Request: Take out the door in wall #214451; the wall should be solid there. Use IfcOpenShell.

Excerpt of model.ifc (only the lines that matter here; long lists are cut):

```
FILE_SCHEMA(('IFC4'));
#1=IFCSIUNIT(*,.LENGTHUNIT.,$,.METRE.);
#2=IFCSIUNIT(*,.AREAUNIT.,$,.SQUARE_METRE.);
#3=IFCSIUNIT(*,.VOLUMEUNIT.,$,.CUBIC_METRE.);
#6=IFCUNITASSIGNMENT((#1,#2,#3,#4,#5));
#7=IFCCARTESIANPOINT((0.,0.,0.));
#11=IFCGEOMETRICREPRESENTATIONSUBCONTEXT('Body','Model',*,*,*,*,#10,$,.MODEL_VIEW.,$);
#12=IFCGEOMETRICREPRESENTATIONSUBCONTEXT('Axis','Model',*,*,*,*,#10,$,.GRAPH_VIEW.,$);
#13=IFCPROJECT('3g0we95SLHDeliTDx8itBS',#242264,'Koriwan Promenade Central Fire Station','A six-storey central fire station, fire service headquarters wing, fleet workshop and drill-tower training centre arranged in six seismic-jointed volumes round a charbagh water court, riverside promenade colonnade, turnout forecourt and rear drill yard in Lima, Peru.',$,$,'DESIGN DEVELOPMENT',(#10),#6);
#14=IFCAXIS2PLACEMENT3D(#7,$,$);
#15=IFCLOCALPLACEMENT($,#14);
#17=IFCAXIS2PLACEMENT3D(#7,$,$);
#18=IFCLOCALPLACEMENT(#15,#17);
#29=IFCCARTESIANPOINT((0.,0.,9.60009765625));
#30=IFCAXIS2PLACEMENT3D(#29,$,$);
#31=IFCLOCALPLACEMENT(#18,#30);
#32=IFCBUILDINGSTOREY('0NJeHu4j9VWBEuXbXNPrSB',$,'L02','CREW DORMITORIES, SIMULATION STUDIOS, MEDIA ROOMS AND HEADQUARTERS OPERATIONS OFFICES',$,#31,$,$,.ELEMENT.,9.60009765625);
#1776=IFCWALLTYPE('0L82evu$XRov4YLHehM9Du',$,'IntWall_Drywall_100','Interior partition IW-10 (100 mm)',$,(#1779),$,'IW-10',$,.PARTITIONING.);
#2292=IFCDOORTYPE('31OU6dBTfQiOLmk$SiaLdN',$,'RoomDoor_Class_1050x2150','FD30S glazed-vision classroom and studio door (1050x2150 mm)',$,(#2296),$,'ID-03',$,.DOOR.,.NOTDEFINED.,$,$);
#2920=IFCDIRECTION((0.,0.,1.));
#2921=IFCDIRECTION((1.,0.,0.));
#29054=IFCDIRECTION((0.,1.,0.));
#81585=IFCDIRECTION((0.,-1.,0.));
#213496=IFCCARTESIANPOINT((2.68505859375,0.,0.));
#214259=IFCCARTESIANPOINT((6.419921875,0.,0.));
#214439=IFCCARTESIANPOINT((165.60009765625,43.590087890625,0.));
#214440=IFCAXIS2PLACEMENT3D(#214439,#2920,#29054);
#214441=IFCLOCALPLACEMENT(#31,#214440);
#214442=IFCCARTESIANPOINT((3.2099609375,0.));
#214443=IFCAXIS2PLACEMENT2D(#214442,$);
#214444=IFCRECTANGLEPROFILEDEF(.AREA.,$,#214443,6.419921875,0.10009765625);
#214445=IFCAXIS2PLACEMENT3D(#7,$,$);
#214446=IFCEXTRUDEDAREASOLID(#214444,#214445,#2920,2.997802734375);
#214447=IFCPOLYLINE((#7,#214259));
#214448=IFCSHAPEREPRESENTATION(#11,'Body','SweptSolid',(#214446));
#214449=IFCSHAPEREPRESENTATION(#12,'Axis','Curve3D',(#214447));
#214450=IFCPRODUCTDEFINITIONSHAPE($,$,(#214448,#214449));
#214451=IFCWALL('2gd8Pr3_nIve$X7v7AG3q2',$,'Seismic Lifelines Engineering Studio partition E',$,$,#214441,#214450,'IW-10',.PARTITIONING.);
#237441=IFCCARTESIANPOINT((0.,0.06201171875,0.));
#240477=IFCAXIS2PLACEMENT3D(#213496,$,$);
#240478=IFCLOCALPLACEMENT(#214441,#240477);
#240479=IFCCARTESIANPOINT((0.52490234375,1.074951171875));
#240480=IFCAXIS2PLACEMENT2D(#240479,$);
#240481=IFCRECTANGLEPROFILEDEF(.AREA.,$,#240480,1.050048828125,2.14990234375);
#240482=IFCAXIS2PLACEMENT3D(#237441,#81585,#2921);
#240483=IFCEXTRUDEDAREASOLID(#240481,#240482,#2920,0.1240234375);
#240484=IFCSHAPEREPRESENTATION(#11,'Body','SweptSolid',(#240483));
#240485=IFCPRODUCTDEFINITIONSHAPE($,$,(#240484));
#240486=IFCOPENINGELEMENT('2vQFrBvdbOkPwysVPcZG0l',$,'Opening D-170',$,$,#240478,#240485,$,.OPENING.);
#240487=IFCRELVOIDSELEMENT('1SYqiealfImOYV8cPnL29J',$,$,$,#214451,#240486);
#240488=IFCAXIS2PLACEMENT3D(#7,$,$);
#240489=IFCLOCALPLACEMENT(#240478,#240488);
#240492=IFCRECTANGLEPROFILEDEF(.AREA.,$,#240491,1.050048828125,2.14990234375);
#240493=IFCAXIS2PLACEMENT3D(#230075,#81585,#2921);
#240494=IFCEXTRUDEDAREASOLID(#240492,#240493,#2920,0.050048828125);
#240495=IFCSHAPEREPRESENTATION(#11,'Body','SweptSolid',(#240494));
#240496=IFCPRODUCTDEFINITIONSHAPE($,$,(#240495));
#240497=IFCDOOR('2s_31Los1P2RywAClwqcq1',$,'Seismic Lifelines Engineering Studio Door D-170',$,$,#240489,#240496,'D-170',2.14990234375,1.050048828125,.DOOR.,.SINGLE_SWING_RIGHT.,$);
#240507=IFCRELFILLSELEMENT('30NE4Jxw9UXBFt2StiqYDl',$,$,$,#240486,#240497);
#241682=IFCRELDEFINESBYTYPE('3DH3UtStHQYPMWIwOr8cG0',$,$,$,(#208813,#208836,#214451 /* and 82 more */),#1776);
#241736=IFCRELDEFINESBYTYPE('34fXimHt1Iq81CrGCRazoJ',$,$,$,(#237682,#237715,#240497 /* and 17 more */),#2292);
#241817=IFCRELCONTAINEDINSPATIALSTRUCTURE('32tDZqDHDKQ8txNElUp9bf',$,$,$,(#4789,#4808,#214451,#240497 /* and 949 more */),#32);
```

```python
import ifcopenshell
import ifcopenshell.api.feature
import ifcopenshell.api.root
import ifcopenshell.geom
import ifcopenshell.util.shape

model = ifcopenshell.open("model.ifc")
settings = ifcopenshell.geom.settings()


def volume(element):
    """Net volume in cubic metres, openings subtracted."""
    shape = ifcopenshell.geom.create_shape(settings, element)
    return ifcopenshell.util.shape.get_volume(shape.geometry)


door = model.by_guid("2s_31Los1P2RywAClwqcq1")
opening = door.FillsVoids[0].RelatingOpeningElement
wall = opening.VoidsElements[0].RelatingBuildingElement
before = volume(wall)

ifcopenshell.api.root.remove_product(model, product=door)
ifcopenshell.api.feature.remove_feature(model, feature=opening)

after = volume(wall)

print(f"wall volume {before:.3f} -> {after:.3f} m3")

model.write("model_edited.ifc")
```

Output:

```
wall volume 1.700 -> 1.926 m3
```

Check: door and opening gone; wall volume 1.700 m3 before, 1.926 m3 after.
